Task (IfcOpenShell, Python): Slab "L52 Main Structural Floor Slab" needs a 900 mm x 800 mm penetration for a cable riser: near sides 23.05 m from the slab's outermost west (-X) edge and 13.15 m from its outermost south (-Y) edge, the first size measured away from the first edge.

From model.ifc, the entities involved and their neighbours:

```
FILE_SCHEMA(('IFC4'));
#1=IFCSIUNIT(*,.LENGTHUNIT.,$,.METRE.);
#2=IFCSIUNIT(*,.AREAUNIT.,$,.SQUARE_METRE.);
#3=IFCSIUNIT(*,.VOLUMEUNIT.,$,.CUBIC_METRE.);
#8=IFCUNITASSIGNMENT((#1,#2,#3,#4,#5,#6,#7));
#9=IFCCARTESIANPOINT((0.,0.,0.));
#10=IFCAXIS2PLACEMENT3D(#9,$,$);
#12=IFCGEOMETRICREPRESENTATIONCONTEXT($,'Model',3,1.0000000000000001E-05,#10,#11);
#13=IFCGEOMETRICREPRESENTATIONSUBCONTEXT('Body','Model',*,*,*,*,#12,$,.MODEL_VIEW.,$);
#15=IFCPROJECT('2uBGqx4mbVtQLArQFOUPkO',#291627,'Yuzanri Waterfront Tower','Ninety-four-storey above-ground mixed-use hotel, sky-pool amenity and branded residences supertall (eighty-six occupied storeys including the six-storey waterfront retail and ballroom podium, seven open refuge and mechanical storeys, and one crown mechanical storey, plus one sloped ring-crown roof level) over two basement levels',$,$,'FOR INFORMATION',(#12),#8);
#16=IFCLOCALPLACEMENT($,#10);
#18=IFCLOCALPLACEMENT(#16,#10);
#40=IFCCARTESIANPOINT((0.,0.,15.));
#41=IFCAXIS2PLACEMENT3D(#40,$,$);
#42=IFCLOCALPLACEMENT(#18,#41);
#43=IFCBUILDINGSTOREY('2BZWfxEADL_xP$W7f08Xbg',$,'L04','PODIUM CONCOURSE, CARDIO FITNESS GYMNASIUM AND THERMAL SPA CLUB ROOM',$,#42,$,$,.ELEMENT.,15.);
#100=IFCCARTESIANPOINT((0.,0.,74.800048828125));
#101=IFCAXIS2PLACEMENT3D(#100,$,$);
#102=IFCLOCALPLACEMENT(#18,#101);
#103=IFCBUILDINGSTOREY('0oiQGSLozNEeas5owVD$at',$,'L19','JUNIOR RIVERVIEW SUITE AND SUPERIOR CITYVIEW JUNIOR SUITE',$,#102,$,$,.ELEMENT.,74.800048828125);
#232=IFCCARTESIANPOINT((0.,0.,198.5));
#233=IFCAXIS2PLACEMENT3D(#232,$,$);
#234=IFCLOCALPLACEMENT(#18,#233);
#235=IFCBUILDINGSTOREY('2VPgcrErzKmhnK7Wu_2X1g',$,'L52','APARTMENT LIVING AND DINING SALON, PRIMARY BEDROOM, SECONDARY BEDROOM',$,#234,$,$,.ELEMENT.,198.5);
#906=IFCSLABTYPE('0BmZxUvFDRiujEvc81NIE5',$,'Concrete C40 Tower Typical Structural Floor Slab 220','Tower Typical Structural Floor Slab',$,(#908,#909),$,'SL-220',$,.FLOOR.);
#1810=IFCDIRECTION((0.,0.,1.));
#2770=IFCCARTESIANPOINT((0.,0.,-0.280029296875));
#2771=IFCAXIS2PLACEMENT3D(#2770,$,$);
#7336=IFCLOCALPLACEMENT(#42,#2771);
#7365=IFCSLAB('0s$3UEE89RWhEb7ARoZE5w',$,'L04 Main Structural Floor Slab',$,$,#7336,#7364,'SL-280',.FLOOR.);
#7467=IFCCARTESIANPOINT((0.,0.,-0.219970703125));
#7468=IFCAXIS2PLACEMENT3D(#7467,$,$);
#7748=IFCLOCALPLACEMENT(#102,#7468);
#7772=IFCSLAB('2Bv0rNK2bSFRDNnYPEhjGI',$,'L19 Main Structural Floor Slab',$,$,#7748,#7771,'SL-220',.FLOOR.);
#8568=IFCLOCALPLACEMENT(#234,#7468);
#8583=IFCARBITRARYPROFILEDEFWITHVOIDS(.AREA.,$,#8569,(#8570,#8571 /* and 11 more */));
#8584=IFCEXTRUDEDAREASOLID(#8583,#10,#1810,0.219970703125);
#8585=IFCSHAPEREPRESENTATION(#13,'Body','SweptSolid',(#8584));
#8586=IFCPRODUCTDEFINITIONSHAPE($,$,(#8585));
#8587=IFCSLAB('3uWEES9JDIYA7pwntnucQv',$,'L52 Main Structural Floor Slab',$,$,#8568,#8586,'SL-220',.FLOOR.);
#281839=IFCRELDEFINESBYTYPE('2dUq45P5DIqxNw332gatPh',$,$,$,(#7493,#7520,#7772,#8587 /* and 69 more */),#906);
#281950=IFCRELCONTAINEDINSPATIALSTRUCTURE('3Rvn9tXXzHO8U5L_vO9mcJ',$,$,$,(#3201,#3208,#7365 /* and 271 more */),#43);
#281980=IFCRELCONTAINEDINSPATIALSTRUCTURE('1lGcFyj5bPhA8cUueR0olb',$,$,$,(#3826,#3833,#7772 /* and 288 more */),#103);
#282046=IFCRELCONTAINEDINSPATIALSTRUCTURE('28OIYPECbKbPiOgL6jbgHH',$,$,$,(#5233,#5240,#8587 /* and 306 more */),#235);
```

```python
import numpy as np
import ifcopenshell
import ifcopenshell.api.feature
import ifcopenshell.api.geometry
import ifcopenshell.api.root
import ifcopenshell.geom
import ifcopenshell.util.placement
import ifcopenshell.util.representation
import ifcopenshell.util.shape
import ifcopenshell.util.unit

model = ifcopenshell.open("model.ifc")
unit_scale = ifcopenshell.util.unit.calculate_unit_scale(model)
settings = ifcopenshell.geom.settings()


def volume(element):
    """Net volume in cubic metres, openings subtracted."""
    shape = ifcopenshell.geom.create_shape(settings, element)
    return ifcopenshell.util.shape.get_volume(shape.geometry)


slab = model.by_guid("3uWEES9JDIYA7pwntnucQv")
before = volume(slab)

# Extent in the slab's own axes, in metres. The edges named are its -X and -Y sides.
slab_shape = ifcopenshell.geom.create_shape(settings, slab)
vertices = ifcopenshell.util.shape.get_vertices(slab_shape.geometry)
x_min, y_min, bottom = vertices.min(axis=0)
top = vertices[:, 2].max()

opening = ifcopenshell.api.root.create_entity(model, ifc_class="IfcOpeningElement", name="Cable riser opening", predefined_type="OPENING")
context = ifcopenshell.util.representation.get_context(model, "Model", "Body", "MODEL_VIEW")
width, depth = 0.9, 0.8
outline = [(0.0, 0.0), (width, 0.0), (width, depth), (0.0, depth), (0.0, 0.0)]
# Overshoot both faces by 50 mm so the cut is clean.
shape = ifcopenshell.api.geometry.add_slab_representation(
    model, context=context, depth=top - bottom + 0.1, polyline=outline
)
ifcopenshell.api.geometry.assign_representation(model, product=opening, representation=shape)

matrix = ifcopenshell.util.placement.get_local_placement(slab.ObjectPlacement)
matrix[:, 3] = matrix @ np.append(np.array([x_min + 23.05, y_min + 13.15, bottom - 0.05]) / unit_scale, 1.0)
ifcopenshell.api.geometry.edit_object_placement(model, product=opening, matrix=matrix, is_si=False)
ifcopenshell.api.feature.add_feature(model, feature=opening, element=slab)

after = volume(slab)

print(f"slab volume {before:.3f} -> {after:.3f} m3")

model.write("model_edited.ifc")
```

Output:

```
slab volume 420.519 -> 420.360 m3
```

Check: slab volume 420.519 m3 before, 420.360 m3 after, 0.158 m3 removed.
